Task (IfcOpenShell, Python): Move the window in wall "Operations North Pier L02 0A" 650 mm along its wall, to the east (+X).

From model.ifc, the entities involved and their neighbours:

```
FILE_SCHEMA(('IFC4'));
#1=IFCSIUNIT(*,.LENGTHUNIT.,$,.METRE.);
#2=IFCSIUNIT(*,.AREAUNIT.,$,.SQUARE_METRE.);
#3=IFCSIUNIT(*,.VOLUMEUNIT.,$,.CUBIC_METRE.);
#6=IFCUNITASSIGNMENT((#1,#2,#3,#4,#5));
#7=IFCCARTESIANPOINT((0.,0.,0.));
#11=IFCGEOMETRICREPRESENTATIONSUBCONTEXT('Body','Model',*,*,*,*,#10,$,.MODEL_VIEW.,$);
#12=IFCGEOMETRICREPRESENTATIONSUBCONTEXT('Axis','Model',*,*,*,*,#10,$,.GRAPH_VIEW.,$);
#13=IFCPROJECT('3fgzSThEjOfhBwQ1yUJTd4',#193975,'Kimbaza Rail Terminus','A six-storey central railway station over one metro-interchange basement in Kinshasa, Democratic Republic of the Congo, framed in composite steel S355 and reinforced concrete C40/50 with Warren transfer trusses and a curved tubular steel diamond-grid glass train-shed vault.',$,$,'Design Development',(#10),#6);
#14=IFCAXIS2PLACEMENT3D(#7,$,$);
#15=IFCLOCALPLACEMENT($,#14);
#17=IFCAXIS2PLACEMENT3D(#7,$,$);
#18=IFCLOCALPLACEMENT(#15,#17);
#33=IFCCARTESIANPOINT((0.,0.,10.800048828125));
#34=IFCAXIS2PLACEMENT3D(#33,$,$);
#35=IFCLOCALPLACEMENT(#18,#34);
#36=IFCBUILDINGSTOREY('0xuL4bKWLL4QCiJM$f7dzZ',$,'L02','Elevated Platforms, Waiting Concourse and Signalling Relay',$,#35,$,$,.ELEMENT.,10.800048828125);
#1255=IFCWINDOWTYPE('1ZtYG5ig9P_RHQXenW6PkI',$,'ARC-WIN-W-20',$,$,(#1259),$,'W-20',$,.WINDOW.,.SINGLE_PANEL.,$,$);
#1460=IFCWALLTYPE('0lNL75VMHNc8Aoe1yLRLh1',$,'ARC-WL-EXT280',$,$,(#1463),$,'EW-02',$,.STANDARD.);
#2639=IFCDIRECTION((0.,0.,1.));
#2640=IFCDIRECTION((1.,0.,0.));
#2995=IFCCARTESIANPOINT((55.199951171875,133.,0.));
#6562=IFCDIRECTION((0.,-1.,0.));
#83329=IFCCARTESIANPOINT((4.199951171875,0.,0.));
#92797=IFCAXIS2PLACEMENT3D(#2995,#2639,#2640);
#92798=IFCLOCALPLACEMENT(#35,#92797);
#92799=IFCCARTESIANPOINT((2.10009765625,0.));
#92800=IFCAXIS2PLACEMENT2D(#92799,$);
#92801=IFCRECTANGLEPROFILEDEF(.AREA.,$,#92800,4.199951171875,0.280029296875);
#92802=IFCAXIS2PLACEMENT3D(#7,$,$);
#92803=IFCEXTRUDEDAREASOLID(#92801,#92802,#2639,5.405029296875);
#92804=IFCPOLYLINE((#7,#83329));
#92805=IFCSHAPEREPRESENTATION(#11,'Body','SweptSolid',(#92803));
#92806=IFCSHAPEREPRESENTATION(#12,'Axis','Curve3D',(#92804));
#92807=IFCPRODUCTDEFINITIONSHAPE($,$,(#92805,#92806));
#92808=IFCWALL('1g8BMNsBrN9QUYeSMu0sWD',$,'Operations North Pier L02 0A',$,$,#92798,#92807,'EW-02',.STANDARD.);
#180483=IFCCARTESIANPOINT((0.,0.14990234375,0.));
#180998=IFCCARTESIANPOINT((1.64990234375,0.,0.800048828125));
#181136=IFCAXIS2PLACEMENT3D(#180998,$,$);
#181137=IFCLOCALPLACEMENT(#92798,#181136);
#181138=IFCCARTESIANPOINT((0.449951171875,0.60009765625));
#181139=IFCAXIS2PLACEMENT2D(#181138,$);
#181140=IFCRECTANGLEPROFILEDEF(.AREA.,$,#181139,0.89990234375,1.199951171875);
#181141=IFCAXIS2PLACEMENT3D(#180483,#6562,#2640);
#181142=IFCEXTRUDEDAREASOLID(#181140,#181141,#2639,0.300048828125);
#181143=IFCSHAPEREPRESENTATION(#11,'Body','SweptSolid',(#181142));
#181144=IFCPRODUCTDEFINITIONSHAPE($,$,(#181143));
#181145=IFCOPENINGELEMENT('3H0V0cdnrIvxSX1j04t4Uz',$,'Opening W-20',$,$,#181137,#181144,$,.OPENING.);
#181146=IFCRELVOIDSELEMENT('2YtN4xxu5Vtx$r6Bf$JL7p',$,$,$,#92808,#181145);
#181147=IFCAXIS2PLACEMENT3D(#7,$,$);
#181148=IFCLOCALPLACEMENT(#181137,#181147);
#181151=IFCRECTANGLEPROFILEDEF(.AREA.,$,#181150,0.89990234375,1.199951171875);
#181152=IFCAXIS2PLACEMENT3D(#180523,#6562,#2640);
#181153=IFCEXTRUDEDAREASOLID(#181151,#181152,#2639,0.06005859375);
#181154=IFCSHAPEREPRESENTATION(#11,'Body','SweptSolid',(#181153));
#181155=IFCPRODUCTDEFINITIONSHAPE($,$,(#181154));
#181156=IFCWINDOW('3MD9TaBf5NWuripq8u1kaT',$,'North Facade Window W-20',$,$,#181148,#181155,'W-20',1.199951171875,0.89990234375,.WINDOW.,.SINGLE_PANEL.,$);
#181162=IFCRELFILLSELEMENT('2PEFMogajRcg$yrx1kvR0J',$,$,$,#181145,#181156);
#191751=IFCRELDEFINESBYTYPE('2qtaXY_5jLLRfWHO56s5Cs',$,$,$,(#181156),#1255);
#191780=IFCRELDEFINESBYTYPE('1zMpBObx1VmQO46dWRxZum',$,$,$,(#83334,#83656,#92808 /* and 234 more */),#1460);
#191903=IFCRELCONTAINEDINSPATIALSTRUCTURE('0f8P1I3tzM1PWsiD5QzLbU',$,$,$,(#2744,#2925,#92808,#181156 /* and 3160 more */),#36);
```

```python
import ifcopenshell
import ifcopenshell.api.geometry
import ifcopenshell.util.placement
import ifcopenshell.util.unit

model = ifcopenshell.open("model.ifc")
unit_scale = ifcopenshell.util.unit.calculate_unit_scale(model)

window = model.by_guid("3MD9TaBf5NWuripq8u1kaT")
opening = window.FillsVoids[0].RelatingOpeningElement
wall = opening.VoidsElements[0].RelatingBuildingElement

wall_matrix = ifcopenshell.util.placement.get_local_placement(wall.ObjectPlacement)
shift = wall_matrix[:3, 0] * 0.65 / unit_scale
before = ifcopenshell.util.placement.get_local_placement(window.ObjectPlacement)[:3, 3].copy()

# The window is placed relative to its opening, so it follows when the opening moves.
matrix = ifcopenshell.util.placement.get_local_placement(opening.ObjectPlacement)
matrix[:3, 3] += shift
ifcopenshell.api.geometry.edit_object_placement(
    model, product=opening, matrix=matrix, is_si=False, should_transform_children=True
)

after = ifcopenshell.util.placement.get_local_placement(window.ObjectPlacement)[:3, 3]
print("window moved by", (after - before).round(3) + 0.0)

model.write("model-out.ifc")
```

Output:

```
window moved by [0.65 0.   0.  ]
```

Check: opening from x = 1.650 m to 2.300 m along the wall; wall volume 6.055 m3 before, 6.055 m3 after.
